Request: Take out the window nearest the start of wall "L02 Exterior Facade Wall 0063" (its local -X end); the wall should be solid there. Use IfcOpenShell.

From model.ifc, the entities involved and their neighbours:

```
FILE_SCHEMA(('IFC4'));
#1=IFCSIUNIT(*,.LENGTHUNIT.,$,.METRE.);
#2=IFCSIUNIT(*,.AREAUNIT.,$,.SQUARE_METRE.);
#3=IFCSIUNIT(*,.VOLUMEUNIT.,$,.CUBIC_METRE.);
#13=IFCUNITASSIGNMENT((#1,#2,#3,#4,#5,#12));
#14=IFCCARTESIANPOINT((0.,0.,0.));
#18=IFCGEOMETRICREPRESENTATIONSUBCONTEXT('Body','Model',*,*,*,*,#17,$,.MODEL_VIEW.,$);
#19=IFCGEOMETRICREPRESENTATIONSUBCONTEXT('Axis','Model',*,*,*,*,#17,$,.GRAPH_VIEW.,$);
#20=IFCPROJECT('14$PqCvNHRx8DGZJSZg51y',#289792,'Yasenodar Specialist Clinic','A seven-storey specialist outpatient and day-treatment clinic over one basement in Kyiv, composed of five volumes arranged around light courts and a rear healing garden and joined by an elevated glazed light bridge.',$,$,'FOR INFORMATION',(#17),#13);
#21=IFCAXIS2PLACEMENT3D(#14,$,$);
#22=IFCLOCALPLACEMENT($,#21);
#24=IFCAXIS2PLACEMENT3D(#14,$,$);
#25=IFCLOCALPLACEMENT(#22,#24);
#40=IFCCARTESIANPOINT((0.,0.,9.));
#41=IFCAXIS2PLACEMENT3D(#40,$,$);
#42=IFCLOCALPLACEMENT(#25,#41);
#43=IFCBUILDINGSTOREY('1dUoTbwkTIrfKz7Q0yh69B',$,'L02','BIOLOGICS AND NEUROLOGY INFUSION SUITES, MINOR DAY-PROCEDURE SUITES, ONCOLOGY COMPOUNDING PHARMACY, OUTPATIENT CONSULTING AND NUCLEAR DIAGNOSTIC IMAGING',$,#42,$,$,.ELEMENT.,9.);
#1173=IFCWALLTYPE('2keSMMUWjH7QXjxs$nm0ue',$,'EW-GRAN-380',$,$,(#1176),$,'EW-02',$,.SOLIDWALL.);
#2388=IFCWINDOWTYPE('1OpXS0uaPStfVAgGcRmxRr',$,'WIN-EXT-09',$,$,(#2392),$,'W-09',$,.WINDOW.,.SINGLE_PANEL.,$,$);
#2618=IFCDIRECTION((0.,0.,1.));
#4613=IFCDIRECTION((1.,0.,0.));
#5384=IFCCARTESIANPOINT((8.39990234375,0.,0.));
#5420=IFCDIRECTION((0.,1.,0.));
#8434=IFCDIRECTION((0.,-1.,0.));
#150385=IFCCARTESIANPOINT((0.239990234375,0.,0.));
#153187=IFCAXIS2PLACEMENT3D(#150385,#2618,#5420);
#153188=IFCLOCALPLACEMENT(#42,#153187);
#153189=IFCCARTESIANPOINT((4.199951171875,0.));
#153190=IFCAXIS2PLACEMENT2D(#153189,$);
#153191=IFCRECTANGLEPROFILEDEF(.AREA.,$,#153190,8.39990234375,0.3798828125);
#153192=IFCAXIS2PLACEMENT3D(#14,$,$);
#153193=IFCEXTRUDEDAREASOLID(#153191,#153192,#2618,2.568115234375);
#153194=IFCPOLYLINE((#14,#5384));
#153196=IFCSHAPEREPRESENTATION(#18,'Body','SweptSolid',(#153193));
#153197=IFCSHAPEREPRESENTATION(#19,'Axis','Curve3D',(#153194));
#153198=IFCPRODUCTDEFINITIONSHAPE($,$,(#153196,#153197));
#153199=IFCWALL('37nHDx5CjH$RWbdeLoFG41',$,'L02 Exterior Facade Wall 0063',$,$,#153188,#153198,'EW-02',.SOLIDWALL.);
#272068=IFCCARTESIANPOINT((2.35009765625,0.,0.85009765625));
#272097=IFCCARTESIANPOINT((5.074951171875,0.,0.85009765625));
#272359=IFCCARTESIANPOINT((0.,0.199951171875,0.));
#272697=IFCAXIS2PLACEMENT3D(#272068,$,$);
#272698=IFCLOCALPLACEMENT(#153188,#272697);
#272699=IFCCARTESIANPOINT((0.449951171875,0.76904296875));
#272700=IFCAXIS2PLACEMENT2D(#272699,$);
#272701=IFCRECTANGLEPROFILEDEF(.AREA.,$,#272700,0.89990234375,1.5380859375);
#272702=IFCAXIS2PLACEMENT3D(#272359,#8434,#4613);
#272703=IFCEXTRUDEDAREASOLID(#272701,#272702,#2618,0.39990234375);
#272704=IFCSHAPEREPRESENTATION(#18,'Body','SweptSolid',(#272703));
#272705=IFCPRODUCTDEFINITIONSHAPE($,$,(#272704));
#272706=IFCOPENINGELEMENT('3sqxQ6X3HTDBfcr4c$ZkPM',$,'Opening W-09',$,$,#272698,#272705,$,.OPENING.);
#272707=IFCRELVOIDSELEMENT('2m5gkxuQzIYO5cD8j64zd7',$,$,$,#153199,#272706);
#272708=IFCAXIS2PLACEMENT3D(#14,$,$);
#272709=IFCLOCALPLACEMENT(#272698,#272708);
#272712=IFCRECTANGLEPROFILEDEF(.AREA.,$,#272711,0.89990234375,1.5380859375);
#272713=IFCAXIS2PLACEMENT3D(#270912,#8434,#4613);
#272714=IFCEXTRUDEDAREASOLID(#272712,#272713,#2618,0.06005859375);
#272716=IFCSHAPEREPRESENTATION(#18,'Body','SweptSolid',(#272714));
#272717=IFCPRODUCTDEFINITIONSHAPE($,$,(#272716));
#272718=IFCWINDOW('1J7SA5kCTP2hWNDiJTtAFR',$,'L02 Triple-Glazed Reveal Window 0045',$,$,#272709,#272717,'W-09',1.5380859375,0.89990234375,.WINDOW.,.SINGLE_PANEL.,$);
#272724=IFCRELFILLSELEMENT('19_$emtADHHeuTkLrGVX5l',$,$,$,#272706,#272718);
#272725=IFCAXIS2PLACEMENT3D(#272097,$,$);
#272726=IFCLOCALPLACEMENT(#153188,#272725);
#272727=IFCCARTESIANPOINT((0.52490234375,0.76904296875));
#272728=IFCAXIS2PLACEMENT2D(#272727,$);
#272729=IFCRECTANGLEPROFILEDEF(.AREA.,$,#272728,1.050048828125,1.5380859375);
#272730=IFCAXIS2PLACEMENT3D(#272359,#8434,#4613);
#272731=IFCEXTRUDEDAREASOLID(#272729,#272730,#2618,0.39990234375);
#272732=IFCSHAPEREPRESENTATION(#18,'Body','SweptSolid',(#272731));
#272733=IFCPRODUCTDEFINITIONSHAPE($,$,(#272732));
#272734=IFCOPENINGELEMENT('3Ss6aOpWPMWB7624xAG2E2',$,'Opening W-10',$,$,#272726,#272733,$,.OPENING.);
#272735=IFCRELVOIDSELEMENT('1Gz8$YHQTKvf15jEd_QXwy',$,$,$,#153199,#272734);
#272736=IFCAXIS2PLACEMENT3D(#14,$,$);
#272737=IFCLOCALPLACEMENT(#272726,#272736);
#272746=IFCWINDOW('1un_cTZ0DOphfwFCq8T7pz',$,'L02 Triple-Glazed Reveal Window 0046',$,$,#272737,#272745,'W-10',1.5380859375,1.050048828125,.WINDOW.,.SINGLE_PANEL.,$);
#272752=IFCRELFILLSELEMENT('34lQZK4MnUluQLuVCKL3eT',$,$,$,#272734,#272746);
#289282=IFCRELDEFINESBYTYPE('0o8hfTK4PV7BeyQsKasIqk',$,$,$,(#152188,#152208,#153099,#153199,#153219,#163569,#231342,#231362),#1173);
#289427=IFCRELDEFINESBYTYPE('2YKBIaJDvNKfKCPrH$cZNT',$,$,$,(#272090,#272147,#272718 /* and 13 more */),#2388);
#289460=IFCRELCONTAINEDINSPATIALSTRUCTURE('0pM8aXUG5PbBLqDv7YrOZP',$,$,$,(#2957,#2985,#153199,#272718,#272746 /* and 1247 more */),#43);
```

```python
import ifcopenshell
import ifcopenshell.api.feature
import ifcopenshell.api.root
import ifcopenshell.geom
import ifcopenshell.util.shape

model = ifcopenshell.open("model.ifc")
settings = ifcopenshell.geom.settings()


def volume(element):
    """Net volume in cubic metres, openings subtracted."""
    shape = ifcopenshell.geom.create_shape(settings, element)
    return ifcopenshell.util.shape.get_volume(shape.geometry)


window = model.by_guid("1J7SA5kCTP2hWNDiJTtAFR")
opening = window.FillsVoids[0].RelatingOpeningElement
wall = opening.VoidsElements[0].RelatingBuildingElement
before = volume(wall)

ifcopenshell.api.root.remove_product(model, product=window)
ifcopenshell.api.feature.remove_feature(model, feature=opening)

after = volume(wall)

print(f"wall volume {before:.3f} -> {after:.3f} m3")

model.write("model_rev.ifc")
```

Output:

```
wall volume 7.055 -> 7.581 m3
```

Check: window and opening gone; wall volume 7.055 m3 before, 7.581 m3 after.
